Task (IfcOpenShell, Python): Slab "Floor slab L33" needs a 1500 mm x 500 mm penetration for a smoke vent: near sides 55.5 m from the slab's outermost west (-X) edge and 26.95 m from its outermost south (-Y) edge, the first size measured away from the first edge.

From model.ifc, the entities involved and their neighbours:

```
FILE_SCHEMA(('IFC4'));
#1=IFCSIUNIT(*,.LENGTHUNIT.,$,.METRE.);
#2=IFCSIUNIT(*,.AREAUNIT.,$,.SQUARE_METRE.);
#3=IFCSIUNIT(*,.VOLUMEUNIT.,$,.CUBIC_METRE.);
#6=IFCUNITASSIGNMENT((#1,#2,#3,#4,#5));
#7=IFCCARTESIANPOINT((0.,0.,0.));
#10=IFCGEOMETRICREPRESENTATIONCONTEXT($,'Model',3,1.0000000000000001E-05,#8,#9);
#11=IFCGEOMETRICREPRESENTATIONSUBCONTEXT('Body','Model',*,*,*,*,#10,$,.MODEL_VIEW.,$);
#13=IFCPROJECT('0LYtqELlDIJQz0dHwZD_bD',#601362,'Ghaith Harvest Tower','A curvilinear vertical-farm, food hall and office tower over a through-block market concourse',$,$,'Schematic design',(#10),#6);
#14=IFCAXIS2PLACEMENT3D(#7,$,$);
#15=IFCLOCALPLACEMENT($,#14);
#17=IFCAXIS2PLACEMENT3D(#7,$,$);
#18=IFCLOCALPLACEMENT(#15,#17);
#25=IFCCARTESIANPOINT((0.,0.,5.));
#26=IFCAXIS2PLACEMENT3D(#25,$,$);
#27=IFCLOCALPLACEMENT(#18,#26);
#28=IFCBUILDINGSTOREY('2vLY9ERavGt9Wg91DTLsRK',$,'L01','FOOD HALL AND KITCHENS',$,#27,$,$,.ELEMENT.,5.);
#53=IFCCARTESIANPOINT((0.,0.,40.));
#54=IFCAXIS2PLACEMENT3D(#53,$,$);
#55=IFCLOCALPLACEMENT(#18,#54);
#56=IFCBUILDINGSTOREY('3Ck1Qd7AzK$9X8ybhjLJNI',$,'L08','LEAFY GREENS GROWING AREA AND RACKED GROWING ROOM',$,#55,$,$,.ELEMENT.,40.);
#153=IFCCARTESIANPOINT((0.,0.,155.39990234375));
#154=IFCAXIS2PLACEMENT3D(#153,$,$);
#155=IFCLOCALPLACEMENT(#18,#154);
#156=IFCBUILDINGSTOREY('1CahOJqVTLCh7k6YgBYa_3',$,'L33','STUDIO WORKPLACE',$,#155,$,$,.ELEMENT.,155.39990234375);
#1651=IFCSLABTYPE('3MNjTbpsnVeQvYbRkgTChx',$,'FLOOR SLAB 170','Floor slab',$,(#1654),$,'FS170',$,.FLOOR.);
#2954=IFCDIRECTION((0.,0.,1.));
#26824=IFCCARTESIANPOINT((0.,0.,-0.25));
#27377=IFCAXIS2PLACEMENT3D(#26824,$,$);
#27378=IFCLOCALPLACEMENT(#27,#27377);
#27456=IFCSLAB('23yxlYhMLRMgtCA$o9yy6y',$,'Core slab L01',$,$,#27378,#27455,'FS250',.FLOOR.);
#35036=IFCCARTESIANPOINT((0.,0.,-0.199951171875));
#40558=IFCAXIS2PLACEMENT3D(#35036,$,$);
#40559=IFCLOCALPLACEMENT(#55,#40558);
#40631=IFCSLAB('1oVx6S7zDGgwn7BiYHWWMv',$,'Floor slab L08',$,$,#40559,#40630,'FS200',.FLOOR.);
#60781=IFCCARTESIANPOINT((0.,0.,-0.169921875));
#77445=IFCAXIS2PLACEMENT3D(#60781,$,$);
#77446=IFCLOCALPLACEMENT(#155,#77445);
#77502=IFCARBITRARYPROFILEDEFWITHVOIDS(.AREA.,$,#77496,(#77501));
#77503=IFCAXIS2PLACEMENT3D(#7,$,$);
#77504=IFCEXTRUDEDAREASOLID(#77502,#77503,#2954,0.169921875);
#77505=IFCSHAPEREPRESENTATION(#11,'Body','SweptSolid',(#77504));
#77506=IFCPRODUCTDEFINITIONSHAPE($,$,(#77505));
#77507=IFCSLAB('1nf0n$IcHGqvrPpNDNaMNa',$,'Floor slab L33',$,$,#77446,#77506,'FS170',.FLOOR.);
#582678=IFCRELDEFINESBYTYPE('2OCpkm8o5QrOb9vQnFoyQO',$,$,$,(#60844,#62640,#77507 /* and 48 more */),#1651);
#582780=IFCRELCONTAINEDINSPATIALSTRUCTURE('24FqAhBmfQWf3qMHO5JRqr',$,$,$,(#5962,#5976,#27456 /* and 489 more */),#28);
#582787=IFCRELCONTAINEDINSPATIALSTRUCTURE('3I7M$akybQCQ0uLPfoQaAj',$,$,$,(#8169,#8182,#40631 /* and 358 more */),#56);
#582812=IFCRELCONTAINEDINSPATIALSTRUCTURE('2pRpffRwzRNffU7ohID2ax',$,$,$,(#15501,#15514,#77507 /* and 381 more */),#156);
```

```python
import numpy as np
import ifcopenshell
import ifcopenshell.api.feature
import ifcopenshell.api.geometry
import ifcopenshell.api.root
import ifcopenshell.geom
import ifcopenshell.util.placement
import ifcopenshell.util.representation
import ifcopenshell.util.shape
import ifcopenshell.util.unit

model = ifcopenshell.open("model.ifc")
unit_scale = ifcopenshell.util.unit.calculate_unit_scale(model)
settings = ifcopenshell.geom.settings()


def volume(element):
    """Net volume in cubic metres, openings subtracted."""
    shape = ifcopenshell.geom.create_shape(settings, element)
    return ifcopenshell.util.shape.get_volume(shape.geometry)


slab = model.by_id(77507)
before = volume(slab)

# Extent in the slab's own axes, in metres. The edges named are its -X and -Y sides.
slab_shape = ifcopenshell.geom.create_shape(settings, slab)
vertices = ifcopenshell.util.shape.get_vertices(slab_shape.geometry)
x_min, y_min, bottom = vertices.min(axis=0)
top = vertices[:, 2].max()

opening = ifcopenshell.api.root.create_entity(model, ifc_class="IfcOpeningElement", name="Smoke vent opening", predefined_type="OPENING")
context = ifcopenshell.util.representation.get_context(model, "Model", "Body", "MODEL_VIEW")
width, depth = 1.5, 0.5
outline = [(0.0, 0.0), (width, 0.0), (width, depth), (0.0, depth), (0.0, 0.0)]
# Overshoot both faces by 50 mm so the cut is clean.
shape = ifcopenshell.api.geometry.add_slab_representation(
    model, context=context, depth=top - bottom + 0.1, polyline=outline
)
ifcopenshell.api.geometry.assign_representation(model, product=opening, representation=shape)

matrix = ifcopenshell.util.placement.get_local_placement(slab.ObjectPlacement)
matrix[:, 3] = matrix @ np.append(np.array([x_min + 55.5, y_min + 26.95, bottom - 0.05]) / unit_scale, 1.0)
ifcopenshell.api.geometry.edit_object_placement(model, product=opening, matrix=matrix, is_si=False)
ifcopenshell.api.feature.add_feature(model, feature=opening, element=slab)

after = volume(slab)

print(f"slab volume {before:.3f} -> {after:.3f} m3")

model.write("model_updated.ifc")
```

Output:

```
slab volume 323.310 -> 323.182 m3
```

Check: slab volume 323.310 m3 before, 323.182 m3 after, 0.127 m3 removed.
